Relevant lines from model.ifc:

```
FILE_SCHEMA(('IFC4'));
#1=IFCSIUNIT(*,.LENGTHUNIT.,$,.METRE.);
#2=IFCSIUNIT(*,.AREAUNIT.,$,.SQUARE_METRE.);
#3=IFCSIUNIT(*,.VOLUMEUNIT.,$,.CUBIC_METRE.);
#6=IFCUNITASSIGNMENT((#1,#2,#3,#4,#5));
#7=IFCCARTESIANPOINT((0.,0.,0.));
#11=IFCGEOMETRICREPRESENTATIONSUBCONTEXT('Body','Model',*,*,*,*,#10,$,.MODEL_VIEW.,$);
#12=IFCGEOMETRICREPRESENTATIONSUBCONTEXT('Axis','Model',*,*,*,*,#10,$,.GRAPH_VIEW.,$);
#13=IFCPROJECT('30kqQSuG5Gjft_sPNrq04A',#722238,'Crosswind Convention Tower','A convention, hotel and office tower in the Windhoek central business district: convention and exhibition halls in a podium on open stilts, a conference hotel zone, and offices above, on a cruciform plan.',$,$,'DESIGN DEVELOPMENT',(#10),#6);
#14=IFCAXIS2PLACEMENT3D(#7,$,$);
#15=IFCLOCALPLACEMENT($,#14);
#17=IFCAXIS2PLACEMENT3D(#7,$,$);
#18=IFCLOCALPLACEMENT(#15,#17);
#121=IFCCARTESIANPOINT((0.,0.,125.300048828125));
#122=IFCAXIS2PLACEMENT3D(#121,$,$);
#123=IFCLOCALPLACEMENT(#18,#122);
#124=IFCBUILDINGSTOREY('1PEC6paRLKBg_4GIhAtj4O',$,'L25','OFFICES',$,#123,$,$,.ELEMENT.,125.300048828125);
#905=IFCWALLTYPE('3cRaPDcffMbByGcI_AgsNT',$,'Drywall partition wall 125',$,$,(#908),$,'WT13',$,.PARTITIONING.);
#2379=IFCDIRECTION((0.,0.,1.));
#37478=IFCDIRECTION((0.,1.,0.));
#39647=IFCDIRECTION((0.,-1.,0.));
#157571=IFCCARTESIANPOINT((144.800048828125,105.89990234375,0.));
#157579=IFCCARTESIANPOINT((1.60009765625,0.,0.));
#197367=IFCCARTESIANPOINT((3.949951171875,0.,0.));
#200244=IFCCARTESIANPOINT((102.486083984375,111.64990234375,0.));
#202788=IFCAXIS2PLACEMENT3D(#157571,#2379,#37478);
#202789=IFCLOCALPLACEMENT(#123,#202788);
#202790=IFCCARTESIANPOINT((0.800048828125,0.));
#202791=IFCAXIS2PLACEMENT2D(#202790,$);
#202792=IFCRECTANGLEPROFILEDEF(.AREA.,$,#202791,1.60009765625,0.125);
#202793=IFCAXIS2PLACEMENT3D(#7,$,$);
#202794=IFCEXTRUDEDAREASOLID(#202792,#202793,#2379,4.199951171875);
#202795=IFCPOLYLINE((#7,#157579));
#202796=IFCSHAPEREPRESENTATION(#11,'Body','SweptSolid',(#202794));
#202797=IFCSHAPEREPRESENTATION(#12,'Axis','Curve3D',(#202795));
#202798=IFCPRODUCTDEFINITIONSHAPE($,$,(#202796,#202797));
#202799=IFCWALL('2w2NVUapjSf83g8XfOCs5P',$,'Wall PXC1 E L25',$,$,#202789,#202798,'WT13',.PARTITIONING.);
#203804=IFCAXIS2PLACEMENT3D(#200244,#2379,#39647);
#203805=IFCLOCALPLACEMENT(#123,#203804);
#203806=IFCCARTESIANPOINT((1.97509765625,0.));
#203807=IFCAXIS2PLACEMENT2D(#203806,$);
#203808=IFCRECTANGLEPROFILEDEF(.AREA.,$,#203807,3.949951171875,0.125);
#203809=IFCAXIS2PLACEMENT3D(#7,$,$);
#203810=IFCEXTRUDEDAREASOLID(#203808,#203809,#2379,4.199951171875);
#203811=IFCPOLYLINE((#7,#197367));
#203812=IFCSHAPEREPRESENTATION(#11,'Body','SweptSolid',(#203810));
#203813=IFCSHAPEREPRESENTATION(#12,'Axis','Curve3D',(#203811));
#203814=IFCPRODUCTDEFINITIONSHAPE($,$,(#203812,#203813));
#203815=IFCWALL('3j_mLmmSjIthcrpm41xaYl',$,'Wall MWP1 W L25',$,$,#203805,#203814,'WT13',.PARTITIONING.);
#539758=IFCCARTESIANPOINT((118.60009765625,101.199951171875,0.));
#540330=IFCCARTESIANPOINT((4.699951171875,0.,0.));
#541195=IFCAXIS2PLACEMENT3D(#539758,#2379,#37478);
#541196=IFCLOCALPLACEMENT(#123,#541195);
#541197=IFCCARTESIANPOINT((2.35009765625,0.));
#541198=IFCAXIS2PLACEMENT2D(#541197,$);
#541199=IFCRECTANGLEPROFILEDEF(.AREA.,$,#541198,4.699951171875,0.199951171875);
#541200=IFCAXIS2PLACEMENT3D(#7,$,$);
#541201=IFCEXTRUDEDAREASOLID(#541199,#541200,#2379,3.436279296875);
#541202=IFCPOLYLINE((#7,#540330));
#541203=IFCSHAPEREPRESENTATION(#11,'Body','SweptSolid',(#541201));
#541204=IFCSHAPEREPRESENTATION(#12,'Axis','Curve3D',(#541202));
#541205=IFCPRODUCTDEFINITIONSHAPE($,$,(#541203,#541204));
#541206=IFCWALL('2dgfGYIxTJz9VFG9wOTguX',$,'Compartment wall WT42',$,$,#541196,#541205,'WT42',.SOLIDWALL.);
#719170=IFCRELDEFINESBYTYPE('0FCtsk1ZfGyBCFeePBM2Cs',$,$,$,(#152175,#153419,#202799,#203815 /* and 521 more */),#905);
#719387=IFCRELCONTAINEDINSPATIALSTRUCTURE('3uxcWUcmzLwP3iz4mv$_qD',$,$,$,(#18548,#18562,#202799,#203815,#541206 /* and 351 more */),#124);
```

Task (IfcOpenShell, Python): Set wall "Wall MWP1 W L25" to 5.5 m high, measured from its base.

```python
import ifcopenshell
import ifcopenshell.geom
import ifcopenshell.util.representation
import ifcopenshell.util.shape

model = ifcopenshell.open("model.ifc")
settings = ifcopenshell.geom.settings()


def volume(element):
    """Net volume in cubic metres, openings subtracted."""
    shape = ifcopenshell.geom.create_shape(settings, element)
    return ifcopenshell.util.shape.get_volume(shape.geometry)


wall = model.by_guid("3j_mLmmSjIthcrpm41xaYl")
before = volume(wall)

body = ifcopenshell.util.representation.get_representation(wall, "Model", "Body")
solid = body.Items[0]
old_height = solid.Depth
solid.Depth = 5.5
after = volume(wall)

print(f"height {old_height:g} -> {solid.Depth:g}, volume {before:.3f} -> {after:.3f} m3")

model.write("model_v2.ifc")
```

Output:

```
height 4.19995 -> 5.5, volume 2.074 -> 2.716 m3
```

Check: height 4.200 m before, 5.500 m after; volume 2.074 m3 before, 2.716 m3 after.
